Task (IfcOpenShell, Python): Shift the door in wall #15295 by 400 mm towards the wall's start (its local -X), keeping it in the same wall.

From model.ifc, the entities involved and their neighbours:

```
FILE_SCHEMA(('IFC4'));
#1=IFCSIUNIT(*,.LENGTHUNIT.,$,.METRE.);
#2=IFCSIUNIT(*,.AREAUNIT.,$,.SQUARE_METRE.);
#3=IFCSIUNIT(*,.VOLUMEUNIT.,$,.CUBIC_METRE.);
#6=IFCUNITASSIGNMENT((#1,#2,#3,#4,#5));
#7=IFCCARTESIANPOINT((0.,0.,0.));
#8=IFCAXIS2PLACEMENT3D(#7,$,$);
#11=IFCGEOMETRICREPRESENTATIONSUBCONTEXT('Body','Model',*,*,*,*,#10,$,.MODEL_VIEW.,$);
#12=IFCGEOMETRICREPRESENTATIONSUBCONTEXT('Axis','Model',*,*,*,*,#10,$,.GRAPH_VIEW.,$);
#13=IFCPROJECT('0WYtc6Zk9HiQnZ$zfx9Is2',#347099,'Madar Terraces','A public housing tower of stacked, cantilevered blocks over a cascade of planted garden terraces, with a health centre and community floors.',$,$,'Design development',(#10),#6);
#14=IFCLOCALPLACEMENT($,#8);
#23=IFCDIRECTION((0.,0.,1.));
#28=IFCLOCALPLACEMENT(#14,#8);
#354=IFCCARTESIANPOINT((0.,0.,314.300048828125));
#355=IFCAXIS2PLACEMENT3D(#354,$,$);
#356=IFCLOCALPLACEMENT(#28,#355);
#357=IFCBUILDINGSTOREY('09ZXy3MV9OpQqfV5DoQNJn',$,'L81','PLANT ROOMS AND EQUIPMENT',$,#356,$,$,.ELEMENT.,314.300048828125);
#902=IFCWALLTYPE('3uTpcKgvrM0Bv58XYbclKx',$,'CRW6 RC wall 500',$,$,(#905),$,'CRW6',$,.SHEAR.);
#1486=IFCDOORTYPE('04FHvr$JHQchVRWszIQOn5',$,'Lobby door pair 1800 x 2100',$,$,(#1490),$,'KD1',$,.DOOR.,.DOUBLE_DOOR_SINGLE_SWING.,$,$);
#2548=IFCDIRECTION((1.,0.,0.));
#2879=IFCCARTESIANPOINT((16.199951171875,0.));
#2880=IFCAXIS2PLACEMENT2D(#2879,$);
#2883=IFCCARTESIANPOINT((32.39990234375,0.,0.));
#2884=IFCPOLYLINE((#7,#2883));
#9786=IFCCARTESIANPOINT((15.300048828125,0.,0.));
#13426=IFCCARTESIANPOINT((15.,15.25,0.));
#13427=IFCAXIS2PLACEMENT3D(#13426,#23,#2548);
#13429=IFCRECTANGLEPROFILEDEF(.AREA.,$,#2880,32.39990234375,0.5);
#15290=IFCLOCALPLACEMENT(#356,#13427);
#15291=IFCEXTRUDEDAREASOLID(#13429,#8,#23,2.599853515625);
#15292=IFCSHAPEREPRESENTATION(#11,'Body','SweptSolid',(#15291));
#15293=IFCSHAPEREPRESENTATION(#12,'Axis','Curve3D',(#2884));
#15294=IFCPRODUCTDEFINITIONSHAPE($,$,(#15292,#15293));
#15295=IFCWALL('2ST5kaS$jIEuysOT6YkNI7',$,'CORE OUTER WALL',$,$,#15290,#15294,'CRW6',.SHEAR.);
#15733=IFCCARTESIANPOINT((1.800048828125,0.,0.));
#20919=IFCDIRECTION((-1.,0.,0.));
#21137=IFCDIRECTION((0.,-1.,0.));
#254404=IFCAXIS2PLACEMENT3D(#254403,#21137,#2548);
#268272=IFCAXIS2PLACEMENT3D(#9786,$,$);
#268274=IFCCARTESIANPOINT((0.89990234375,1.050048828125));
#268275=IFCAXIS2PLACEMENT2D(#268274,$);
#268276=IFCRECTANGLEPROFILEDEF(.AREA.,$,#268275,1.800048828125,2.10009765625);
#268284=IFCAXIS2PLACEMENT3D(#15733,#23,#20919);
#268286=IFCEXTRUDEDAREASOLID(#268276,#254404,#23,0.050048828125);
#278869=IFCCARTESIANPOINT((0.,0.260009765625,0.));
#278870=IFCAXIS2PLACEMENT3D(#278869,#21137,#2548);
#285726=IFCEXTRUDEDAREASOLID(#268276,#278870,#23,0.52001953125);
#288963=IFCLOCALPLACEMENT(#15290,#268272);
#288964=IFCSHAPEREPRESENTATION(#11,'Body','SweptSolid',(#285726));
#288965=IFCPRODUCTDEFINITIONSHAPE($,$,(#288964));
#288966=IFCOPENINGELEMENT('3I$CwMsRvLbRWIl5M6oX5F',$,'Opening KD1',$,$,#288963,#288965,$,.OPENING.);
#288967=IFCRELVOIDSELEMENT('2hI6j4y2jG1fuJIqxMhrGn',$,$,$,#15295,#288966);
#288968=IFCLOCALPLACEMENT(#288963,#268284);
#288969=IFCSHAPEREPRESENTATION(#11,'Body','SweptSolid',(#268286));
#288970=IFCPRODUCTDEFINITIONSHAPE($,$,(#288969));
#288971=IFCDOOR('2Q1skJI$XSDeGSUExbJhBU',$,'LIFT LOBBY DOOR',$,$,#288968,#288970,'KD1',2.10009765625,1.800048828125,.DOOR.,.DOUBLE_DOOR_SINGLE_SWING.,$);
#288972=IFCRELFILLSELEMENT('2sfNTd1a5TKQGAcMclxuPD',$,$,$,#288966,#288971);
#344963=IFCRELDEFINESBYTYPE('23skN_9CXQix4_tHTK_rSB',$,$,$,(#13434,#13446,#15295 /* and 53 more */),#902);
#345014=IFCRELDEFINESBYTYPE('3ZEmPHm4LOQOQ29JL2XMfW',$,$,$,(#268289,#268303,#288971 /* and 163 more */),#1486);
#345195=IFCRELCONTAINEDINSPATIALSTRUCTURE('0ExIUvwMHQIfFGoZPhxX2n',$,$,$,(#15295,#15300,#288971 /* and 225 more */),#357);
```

```python
import ifcopenshell
import ifcopenshell.api.geometry
import ifcopenshell.util.placement
import ifcopenshell.util.unit

model = ifcopenshell.open("model.ifc")
unit_scale = ifcopenshell.util.unit.calculate_unit_scale(model)

door = model.by_guid("2Q1skJI$XSDeGSUExbJhBU")
opening = door.FillsVoids[0].RelatingOpeningElement
wall = opening.VoidsElements[0].RelatingBuildingElement

wall_matrix = ifcopenshell.util.placement.get_local_placement(wall.ObjectPlacement)
shift = wall_matrix[:3, 0] * -0.4 / unit_scale
before = ifcopenshell.util.placement.get_local_placement(door.ObjectPlacement)[:3, 3].copy()

# The door is placed relative to its opening, so it follows when the opening moves.
matrix = ifcopenshell.util.placement.get_local_placement(opening.ObjectPlacement)
matrix[:3, 3] += shift
ifcopenshell.api.geometry.edit_object_placement(
    model, product=opening, matrix=matrix, is_si=False, should_transform_children=True
)

after = ifcopenshell.util.placement.get_local_placement(door.ObjectPlacement)[:3, 3]
print("door moved by", (after - before).round(3) + 0.0)

model.write("model-out.ifc")
```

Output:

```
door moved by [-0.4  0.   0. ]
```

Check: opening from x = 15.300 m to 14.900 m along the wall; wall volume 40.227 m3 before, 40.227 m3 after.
